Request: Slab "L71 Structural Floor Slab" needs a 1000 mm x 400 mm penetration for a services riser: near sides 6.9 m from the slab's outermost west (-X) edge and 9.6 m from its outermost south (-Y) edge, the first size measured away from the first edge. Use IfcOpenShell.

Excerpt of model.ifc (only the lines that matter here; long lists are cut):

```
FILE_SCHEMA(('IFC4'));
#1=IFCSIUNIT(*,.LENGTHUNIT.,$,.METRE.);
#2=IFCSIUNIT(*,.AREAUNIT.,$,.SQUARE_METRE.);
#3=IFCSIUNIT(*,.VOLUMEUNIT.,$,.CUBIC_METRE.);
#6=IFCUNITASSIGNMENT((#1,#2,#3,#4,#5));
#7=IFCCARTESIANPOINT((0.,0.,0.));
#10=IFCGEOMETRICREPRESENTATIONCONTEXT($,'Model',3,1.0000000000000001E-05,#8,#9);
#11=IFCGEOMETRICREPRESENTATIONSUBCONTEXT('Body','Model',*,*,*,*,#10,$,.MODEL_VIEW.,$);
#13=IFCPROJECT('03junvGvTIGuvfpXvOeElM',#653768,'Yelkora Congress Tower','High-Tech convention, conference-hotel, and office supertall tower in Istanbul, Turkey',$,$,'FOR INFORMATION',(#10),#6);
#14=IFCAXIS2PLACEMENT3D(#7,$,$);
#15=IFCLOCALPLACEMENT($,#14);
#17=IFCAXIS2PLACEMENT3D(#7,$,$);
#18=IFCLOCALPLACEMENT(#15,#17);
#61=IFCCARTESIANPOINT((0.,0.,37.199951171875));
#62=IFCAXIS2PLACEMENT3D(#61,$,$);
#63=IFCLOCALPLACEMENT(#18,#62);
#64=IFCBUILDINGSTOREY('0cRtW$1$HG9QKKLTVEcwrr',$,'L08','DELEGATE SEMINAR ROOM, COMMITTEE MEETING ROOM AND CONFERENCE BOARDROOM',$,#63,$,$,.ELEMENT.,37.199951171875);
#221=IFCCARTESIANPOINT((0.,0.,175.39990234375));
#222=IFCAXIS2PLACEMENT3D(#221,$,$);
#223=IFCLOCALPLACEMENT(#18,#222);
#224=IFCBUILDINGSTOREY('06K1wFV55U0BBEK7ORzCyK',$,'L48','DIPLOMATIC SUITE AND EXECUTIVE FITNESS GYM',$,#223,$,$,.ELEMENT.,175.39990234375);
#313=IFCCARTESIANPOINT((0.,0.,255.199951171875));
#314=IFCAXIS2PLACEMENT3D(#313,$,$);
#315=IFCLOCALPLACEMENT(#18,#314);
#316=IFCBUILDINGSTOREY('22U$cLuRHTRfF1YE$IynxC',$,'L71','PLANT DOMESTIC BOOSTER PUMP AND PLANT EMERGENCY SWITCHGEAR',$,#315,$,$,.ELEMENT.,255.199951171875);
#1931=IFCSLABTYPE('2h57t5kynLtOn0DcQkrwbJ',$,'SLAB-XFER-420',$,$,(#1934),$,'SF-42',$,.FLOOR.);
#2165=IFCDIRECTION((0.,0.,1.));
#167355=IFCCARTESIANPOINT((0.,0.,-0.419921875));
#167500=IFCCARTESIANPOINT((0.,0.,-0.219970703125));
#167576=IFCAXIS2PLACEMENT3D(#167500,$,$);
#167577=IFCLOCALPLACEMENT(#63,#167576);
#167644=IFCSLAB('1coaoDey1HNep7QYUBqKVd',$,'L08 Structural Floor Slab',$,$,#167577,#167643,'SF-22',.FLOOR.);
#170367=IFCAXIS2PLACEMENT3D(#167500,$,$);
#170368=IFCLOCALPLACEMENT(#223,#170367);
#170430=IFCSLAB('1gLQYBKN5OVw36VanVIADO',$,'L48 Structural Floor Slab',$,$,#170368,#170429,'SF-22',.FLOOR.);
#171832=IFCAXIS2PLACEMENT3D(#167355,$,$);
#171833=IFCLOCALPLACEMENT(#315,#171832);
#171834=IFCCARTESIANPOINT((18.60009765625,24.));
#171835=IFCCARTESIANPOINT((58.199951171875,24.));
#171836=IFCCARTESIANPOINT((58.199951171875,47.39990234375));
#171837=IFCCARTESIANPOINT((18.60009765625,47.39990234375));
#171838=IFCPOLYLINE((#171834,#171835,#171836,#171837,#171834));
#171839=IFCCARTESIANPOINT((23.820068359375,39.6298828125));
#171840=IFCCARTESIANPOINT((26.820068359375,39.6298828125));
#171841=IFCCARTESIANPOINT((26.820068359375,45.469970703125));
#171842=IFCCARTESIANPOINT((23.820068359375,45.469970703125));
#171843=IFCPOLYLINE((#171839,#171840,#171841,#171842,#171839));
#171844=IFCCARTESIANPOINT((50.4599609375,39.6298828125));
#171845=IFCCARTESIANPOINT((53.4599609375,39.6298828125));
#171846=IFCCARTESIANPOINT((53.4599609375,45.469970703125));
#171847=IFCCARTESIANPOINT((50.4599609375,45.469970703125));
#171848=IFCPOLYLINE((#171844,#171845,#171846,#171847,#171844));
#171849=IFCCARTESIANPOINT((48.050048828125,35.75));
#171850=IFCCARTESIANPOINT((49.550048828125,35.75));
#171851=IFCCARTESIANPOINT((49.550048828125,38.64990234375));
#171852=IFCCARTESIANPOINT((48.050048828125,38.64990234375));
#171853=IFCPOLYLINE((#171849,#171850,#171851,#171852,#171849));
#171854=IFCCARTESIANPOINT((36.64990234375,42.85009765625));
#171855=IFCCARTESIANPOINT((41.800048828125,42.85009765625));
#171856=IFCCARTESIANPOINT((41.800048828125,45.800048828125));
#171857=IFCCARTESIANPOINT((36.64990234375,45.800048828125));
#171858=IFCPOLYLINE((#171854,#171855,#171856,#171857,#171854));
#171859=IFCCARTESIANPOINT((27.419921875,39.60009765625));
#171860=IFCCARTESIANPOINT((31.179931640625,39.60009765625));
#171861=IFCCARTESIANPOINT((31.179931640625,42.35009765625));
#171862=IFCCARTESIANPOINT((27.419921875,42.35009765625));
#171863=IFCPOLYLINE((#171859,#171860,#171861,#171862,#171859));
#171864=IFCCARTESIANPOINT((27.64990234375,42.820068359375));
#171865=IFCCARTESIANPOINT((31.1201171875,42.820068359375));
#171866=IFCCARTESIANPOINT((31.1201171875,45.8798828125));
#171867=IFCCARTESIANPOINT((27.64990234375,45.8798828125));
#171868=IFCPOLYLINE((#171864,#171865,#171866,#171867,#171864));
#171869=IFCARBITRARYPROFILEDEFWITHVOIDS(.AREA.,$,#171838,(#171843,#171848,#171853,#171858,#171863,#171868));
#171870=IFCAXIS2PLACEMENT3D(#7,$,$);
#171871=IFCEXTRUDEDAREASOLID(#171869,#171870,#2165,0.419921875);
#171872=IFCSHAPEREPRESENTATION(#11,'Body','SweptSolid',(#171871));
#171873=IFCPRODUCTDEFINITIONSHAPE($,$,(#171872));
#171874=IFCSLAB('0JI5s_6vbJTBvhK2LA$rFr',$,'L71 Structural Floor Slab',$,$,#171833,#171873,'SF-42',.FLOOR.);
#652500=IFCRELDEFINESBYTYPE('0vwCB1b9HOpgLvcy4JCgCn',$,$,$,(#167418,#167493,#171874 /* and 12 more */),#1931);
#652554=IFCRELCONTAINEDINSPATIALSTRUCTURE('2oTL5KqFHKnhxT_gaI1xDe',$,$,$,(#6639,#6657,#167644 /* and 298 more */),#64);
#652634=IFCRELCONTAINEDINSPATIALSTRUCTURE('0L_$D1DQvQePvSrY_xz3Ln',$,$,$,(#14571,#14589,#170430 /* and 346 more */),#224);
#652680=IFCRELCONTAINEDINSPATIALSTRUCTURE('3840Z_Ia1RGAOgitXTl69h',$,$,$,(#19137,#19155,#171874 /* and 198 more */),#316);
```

```python
import numpy as np
import ifcopenshell
import ifcopenshell.api.feature
import ifcopenshell.api.geometry
import ifcopenshell.api.root
import ifcopenshell.geom
import ifcopenshell.util.placement
import ifcopenshell.util.representation
import ifcopenshell.util.shape
import ifcopenshell.util.unit

model = ifcopenshell.open("model.ifc")
unit_scale = ifcopenshell.util.unit.calculate_unit_scale(model)
settings = ifcopenshell.geom.settings()


def volume(element):
    """Net volume in cubic metres, openings subtracted."""
    shape = ifcopenshell.geom.create_shape(settings, element)
    return ifcopenshell.util.shape.get_volume(shape.geometry)


slab = model.by_guid("0JI5s_6vbJTBvhK2LA$rFr")
before = volume(slab)

# Extent in the slab's own axes, in metres. The edges named are its -X and -Y sides.
slab_shape = ifcopenshell.geom.create_shape(settings, slab)
vertices = ifcopenshell.util.shape.get_vertices(slab_shape.geometry)
x_min, y_min, bottom = vertices.min(axis=0)
top = vertices[:, 2].max()

opening = ifcopenshell.api.root.create_entity(model, ifc_class="IfcOpeningElement", name="Services riser opening", predefined_type="OPENING")
context = ifcopenshell.util.representation.get_context(model, "Model", "Body", "MODEL_VIEW")
width, depth = 1, 0.4
outline = [(0.0, 0.0), (width, 0.0), (width, depth), (0.0, depth), (0.0, 0.0)]
# Overshoot both faces by 50 mm so the cut is clean.
shape = ifcopenshell.api.geometry.add_slab_representation(
    model, context=context, depth=top - bottom + 0.1, polyline=outline
)
ifcopenshell.api.geometry.assign_representation(model, product=opening, representation=shape)

matrix = ifcopenshell.util.placement.get_local_placement(slab.ObjectPlacement)
matrix[:, 3] = matrix @ np.append(np.array([x_min + 6.9, y_min + 9.6, bottom - 0.05]) / unit_scale, 1.0)
ifcopenshell.api.geometry.edit_object_placement(model, product=opening, matrix=matrix, is_si=False)
ifcopenshell.api.feature.add_feature(model, feature=opening, element=slab)

after = volume(slab)

print(f"slab volume {before:.3f} -> {after:.3f} m3")

model.write("model_updated.ifc")
```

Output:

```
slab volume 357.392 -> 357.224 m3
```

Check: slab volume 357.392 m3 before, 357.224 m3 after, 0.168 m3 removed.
